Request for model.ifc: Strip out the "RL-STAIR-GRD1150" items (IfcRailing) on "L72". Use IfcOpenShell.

First a look at what the model holds.

```python
import ifcopenshell
import ifcopenshell.util.element

model = ifcopenshell.open("model.ifc")
print(model.schema)
storey = next(s for s in model.by_type("IfcBuildingStorey") if s.Name == "L72")
railings = [e for e in ifcopenshell.util.element.get_decomposition(storey) if e.is_a("IfcRailing")]
seen = {}
for e in railings:
    element_type = ifcopenshell.util.element.get_type(e)
    name = element_type.Name if element_type not in (None, e) else None
    seen[name] = seen.get(name, 0) + 1
for name, count in sorted(seen.items(), key=str):
    print(count, "x", name)
```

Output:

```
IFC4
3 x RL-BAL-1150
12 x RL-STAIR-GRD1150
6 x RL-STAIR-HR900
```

```python
import ifcopenshell
import ifcopenshell.api.root
import ifcopenshell.util.element

model = ifcopenshell.open("model.ifc")

storey = next(s for s in model.by_type("IfcBuildingStorey") if s.Name == "L72")
railings = [e for e in ifcopenshell.util.element.get_decomposition(storey) if e.is_a("IfcRailing")]
targets = [e for e in railings if (t := ifcopenshell.util.element.get_type(e)) not in (None, e) and t.Name == "RL-STAIR-GRD1150"]

for e in targets:
    ifcopenshell.api.root.remove_product(model, product=e)
print(len(targets), "removed")

model.write("model_v2.ifc")
```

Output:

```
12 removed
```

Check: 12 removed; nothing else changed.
